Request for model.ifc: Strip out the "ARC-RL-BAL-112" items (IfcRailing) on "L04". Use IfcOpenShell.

First a look at what the model holds.

```python
import ifcopenshell
import ifcopenshell.util.element

model = ifcopenshell.open("model.ifc")
print(model.schema)
storey = next(s for s in model.by_type("IfcBuildingStorey") if s.Name == "L04")
railings = [e for e in ifcopenshell.util.element.get_decomposition(storey) if e.is_a("IfcRailing")]
seen = {}
for e in railings:
    element_type = ifcopenshell.util.element.get_type(e)
    name = element_type.Name if element_type not in (None, e) else None
    seen[name] = seen.get(name, 0) + 1
for name, count in sorted(seen.items(), key=str):
    print(count, "x", name)
```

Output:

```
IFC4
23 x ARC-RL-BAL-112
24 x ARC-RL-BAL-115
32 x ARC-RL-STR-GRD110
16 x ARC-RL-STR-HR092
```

```python
import ifcopenshell
import ifcopenshell.api.root
import ifcopenshell.util.element

model = ifcopenshell.open("model.ifc")

storey = next(s for s in model.by_type("IfcBuildingStorey") if s.Name == "L04")
railings = [e for e in ifcopenshell.util.element.get_decomposition(storey) if e.is_a("IfcRailing")]
targets = [e for e in railings if (t := ifcopenshell.util.element.get_type(e)) not in (None, e) and t.Name == "ARC-RL-BAL-112"]

for e in targets:
    ifcopenshell.api.root.remove_product(model, product=e)
print(len(targets), "removed")

model.write("model_rev.ifc")
```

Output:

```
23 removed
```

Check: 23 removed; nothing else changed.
